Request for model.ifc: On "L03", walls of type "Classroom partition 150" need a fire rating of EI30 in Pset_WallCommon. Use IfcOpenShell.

First a look at what the model holds.

```python
import ifcopenshell
import ifcopenshell.util.element

model = ifcopenshell.open("model.ifc")
print(model.schema)
storey = next(s for s in model.by_type("IfcBuildingStorey") if s.Name == "L03")
walls = [e for e in ifcopenshell.util.element.get_decomposition(storey) if e.is_a("IfcWall")]
seen = {}
for e in walls:
    element_type = ifcopenshell.util.element.get_type(e)
    key = (element_type.Name if element_type != e and element_type else None, ifcopenshell.util.element.get_pset(e, "Pset_WallCommon", "FireRating"))
    seen[key] = seen.get(key, 0) + 1
for (name, value), count in sorted(seen.items(), key=str):
    print(count, "x", name, "|", value)
```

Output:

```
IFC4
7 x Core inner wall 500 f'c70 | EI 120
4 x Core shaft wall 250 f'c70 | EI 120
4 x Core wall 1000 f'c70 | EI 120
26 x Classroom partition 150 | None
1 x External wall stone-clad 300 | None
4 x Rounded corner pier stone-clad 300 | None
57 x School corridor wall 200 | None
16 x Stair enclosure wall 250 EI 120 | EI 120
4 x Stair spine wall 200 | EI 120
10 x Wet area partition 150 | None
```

```python
import ifcopenshell
import ifcopenshell.api.pset
import ifcopenshell.util.element

model = ifcopenshell.open("model.ifc")

storey = next(s for s in model.by_type("IfcBuildingStorey") if s.Name == "L03")
walls = [e for e in ifcopenshell.util.element.get_decomposition(storey) if e.is_a("IfcWall")]

count = 0
for e in walls:
    element_type = ifcopenshell.util.element.get_type(e)
    if element_type in (None, e) or element_type.Name != "Classroom partition 150":
        continue
    found = ifcopenshell.util.element.get_pset(e, "Pset_WallCommon", should_inherit=False)
    if found:
        pset = model.by_id(found["id"])
        if len(ifcopenshell.util.element.get_elements_by_pset(pset)) > 1:
            pset = ifcopenshell.api.pset.unshare_pset(model, products=[e], pset=pset)[0]
    else:
        pset = ifcopenshell.api.pset.add_pset(model, product=e, name="Pset_WallCommon")
    ifcopenshell.api.pset.edit_pset(model, pset=pset, properties={"FireRating": "EI30"})
    count += 1

print(count, "walls updated")

model.write("model_updated.ifc")
```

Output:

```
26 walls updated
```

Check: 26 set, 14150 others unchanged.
